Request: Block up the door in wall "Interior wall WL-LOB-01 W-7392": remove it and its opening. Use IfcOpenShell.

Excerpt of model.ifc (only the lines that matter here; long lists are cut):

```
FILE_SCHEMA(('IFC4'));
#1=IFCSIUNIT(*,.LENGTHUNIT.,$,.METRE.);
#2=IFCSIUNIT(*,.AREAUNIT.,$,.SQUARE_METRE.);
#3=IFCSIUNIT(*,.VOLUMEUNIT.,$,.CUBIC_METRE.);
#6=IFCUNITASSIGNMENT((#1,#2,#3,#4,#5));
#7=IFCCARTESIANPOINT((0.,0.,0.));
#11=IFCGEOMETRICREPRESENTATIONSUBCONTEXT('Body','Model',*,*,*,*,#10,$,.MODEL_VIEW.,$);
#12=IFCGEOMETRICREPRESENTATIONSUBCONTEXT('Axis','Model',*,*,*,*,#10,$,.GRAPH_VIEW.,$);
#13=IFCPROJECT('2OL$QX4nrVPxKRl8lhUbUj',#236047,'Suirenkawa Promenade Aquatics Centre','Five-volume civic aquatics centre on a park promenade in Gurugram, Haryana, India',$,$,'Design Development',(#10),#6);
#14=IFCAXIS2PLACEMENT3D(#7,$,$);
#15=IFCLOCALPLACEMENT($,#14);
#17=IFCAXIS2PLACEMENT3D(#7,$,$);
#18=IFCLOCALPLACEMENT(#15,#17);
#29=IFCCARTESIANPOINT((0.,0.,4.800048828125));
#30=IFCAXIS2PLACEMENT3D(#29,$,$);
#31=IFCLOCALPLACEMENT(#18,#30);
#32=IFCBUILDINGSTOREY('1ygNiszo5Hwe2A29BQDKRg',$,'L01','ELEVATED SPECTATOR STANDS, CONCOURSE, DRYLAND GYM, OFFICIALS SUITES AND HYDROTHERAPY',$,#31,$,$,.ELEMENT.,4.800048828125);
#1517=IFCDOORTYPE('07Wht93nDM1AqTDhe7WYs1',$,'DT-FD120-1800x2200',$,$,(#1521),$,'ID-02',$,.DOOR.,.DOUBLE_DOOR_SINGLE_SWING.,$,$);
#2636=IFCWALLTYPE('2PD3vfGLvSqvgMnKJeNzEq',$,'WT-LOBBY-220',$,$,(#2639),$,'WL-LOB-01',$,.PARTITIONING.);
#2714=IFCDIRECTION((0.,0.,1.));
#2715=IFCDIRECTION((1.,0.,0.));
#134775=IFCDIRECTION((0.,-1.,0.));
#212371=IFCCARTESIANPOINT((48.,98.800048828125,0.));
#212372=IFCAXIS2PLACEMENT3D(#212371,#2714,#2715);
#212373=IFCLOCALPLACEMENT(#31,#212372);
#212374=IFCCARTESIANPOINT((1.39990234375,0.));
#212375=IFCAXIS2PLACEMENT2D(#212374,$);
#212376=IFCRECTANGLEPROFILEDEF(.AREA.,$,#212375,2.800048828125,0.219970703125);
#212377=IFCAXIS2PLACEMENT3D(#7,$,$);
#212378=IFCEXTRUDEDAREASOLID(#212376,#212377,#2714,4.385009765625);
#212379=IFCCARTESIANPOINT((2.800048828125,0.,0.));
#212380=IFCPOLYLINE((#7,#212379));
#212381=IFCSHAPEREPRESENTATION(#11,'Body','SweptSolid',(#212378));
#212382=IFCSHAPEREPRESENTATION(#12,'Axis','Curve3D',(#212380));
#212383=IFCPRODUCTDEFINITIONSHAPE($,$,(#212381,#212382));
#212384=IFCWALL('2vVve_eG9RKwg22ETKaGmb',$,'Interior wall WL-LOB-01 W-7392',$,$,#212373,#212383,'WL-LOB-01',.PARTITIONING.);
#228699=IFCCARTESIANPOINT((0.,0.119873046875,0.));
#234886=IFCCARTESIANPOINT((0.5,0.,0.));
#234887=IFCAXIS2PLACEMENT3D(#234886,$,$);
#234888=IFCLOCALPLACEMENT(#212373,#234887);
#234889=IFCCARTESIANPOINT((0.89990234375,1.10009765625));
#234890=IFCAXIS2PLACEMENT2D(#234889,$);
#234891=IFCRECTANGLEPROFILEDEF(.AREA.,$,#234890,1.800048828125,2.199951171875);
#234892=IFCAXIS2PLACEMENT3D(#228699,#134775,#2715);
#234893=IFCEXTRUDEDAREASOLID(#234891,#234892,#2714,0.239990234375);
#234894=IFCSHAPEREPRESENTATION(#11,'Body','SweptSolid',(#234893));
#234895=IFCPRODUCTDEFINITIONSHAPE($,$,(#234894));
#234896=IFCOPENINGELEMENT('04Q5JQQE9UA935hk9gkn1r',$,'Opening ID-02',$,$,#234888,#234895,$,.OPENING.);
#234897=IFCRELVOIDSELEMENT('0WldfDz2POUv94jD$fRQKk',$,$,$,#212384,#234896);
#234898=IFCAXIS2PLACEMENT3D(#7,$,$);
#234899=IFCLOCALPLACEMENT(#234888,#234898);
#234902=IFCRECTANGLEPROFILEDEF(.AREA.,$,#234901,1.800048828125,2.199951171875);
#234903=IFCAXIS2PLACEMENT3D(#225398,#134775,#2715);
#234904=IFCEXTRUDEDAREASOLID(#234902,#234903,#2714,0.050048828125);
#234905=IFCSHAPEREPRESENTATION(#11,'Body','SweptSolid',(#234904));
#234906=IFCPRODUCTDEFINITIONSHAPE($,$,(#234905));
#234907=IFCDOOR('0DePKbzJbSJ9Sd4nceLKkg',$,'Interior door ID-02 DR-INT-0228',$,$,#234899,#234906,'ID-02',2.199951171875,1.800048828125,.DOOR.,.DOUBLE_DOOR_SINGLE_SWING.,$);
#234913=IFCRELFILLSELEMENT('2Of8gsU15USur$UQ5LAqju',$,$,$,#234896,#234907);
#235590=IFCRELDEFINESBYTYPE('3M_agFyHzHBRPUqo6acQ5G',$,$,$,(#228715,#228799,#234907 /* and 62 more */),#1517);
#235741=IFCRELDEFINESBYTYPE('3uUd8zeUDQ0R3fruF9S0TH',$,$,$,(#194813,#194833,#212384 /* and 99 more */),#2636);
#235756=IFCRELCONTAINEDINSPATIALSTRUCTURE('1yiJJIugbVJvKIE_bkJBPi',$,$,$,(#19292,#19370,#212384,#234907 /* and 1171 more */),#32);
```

```python
import ifcopenshell
import ifcopenshell.api.feature
import ifcopenshell.api.root
import ifcopenshell.geom
import ifcopenshell.util.shape

model = ifcopenshell.open("model.ifc")
settings = ifcopenshell.geom.settings()


def volume(element):
    """Net volume in cubic metres, openings subtracted."""
    shape = ifcopenshell.geom.create_shape(settings, element)
    return ifcopenshell.util.shape.get_volume(shape.geometry)


door = model.by_guid("0DePKbzJbSJ9Sd4nceLKkg")
opening = door.FillsVoids[0].RelatingOpeningElement
wall = opening.VoidsElements[0].RelatingBuildingElement
before = volume(wall)

ifcopenshell.api.root.remove_product(model, product=door)
ifcopenshell.api.feature.remove_feature(model, feature=opening)

after = volume(wall)

print(f"wall volume {before:.3f} -> {after:.3f} m3")

model.write("model_edited.ifc")
```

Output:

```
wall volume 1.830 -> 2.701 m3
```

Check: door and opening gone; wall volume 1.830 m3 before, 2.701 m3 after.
